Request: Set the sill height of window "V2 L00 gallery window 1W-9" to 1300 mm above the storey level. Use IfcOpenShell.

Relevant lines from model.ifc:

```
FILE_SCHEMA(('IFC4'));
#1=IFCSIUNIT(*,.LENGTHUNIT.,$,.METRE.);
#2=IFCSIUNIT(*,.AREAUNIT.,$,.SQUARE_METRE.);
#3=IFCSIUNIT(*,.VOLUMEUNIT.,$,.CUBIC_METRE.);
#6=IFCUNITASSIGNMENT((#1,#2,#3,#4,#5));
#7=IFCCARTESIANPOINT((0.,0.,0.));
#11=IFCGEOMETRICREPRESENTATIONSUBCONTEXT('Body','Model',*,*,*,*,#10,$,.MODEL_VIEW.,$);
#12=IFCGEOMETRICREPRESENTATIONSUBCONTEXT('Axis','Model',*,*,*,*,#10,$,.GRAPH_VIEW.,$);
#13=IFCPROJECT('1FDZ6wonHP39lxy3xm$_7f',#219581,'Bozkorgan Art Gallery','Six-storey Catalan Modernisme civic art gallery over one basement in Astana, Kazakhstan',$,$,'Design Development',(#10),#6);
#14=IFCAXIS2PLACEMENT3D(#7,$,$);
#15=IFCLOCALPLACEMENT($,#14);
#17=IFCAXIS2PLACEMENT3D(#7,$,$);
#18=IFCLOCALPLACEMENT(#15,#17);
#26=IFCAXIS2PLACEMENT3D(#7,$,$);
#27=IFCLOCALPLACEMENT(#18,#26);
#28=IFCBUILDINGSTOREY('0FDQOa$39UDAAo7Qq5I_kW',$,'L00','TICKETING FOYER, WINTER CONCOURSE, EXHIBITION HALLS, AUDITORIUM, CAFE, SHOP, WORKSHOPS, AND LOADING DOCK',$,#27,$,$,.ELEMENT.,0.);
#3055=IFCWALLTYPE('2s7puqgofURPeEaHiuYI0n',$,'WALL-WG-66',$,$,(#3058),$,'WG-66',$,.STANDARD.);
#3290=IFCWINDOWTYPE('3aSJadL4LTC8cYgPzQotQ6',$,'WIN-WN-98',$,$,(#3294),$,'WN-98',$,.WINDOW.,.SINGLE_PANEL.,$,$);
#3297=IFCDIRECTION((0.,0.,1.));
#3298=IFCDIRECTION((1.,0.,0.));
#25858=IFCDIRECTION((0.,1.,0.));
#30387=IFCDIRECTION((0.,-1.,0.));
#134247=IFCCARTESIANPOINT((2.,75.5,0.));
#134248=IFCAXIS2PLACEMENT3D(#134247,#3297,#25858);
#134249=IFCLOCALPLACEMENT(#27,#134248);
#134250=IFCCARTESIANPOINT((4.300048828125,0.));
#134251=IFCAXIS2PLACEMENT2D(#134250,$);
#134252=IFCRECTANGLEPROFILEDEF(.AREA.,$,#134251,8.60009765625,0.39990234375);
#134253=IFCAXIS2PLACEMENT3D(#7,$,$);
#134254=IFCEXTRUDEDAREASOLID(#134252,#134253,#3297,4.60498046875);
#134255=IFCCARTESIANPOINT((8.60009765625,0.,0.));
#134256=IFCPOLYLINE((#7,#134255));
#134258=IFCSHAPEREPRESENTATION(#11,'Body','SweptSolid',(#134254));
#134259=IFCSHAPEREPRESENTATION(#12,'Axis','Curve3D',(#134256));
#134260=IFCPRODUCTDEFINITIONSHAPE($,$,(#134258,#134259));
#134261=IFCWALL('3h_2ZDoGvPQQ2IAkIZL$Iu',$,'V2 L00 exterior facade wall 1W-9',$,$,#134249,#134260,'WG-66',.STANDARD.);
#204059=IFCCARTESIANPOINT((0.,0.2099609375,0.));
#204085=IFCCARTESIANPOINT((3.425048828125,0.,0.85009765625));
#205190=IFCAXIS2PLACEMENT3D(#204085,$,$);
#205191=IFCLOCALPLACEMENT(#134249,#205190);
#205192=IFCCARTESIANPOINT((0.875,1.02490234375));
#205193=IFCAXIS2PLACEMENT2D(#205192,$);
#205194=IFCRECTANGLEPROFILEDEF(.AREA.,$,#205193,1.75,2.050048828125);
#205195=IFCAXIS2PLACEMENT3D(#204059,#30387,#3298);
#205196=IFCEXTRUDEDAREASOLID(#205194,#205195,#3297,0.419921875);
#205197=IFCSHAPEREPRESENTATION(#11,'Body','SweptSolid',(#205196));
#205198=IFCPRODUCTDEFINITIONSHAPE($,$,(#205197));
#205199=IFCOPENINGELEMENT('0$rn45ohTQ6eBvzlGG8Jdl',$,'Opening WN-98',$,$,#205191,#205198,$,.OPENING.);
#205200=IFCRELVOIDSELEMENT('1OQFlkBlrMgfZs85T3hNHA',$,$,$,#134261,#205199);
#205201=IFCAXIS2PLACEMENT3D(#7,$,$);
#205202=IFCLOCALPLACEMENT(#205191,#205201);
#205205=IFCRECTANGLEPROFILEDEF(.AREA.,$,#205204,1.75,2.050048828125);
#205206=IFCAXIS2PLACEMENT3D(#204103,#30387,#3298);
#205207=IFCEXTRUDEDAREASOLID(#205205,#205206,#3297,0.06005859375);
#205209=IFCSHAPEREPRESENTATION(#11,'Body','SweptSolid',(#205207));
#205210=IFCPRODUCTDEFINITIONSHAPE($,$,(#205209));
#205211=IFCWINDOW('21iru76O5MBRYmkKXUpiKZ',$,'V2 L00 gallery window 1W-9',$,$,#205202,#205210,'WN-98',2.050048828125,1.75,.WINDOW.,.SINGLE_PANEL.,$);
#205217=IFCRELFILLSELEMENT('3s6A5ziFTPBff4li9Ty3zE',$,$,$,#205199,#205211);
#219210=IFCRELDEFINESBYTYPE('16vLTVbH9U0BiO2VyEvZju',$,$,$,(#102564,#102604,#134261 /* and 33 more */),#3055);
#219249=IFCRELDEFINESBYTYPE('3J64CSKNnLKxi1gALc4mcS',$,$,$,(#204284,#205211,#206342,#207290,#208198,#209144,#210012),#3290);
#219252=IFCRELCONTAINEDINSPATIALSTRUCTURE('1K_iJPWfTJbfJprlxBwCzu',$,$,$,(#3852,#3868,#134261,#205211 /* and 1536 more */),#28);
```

```python
import numpy as np
import ifcopenshell
import ifcopenshell.api.geometry
import ifcopenshell.geom
import ifcopenshell.util.element
import ifcopenshell.util.placement
import ifcopenshell.util.shape
import ifcopenshell.util.unit

model = ifcopenshell.open("model.ifc")
unit_scale = ifcopenshell.util.unit.calculate_unit_scale(model)

window = model.by_guid("21iru76O5MBRYmkKXUpiKZ")
opening = window.FillsVoids[0].RelatingOpeningElement
storey = ifcopenshell.util.element.get_container(window, ifc_class="IfcBuildingStorey")
level = ifcopenshell.util.placement.get_local_placement(storey.ObjectPlacement)[2, 3]

# The opening's origin need not be at the sill, so measure its lowest point.
shape = ifcopenshell.geom.create_shape(ifcopenshell.geom.settings(), opening)
bottom = ifcopenshell.util.shape.get_shape_bottom_elevation(shape, shape.geometry) / unit_scale
dz = level + 1.3 - bottom

shift = np.array([0.0, 0.0, dz])
# The window is placed relative to its opening, so it follows when the opening moves.
matrix = ifcopenshell.util.placement.get_local_placement(opening.ObjectPlacement)
matrix[:3, 3] += shift
ifcopenshell.api.geometry.edit_object_placement(
    model, product=opening, matrix=matrix, is_si=False, should_transform_children=True
)

print(f"moved by {dz * unit_scale:+.3f} m")

model.write("model-out.ifc")
```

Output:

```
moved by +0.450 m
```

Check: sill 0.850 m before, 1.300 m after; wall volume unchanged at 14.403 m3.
